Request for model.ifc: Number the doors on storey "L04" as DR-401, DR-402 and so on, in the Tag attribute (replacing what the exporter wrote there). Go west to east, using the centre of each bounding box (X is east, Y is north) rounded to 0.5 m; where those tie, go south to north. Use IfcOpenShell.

First a look at what the model holds.

```python
import ifcopenshell
import ifcopenshell.util.element
import ifcopenshell.util.placement

model = ifcopenshell.open("model.ifc")
print(model.schema)
storey = next(s for s in model.by_type("IfcBuildingStorey") if s.Name == "L04")
doors = [e for e in ifcopenshell.util.element.get_decomposition(storey) if e.is_a("IfcDoor")]
for e in sorted(doors, key=lambda e: e.id()):
    origin = ifcopenshell.util.placement.get_local_placement(e.ObjectPlacement)[:3, 3]
    print(e.id(), e.Tag, e.Name, origin.round(2) + 0.0, sep=" | ")
```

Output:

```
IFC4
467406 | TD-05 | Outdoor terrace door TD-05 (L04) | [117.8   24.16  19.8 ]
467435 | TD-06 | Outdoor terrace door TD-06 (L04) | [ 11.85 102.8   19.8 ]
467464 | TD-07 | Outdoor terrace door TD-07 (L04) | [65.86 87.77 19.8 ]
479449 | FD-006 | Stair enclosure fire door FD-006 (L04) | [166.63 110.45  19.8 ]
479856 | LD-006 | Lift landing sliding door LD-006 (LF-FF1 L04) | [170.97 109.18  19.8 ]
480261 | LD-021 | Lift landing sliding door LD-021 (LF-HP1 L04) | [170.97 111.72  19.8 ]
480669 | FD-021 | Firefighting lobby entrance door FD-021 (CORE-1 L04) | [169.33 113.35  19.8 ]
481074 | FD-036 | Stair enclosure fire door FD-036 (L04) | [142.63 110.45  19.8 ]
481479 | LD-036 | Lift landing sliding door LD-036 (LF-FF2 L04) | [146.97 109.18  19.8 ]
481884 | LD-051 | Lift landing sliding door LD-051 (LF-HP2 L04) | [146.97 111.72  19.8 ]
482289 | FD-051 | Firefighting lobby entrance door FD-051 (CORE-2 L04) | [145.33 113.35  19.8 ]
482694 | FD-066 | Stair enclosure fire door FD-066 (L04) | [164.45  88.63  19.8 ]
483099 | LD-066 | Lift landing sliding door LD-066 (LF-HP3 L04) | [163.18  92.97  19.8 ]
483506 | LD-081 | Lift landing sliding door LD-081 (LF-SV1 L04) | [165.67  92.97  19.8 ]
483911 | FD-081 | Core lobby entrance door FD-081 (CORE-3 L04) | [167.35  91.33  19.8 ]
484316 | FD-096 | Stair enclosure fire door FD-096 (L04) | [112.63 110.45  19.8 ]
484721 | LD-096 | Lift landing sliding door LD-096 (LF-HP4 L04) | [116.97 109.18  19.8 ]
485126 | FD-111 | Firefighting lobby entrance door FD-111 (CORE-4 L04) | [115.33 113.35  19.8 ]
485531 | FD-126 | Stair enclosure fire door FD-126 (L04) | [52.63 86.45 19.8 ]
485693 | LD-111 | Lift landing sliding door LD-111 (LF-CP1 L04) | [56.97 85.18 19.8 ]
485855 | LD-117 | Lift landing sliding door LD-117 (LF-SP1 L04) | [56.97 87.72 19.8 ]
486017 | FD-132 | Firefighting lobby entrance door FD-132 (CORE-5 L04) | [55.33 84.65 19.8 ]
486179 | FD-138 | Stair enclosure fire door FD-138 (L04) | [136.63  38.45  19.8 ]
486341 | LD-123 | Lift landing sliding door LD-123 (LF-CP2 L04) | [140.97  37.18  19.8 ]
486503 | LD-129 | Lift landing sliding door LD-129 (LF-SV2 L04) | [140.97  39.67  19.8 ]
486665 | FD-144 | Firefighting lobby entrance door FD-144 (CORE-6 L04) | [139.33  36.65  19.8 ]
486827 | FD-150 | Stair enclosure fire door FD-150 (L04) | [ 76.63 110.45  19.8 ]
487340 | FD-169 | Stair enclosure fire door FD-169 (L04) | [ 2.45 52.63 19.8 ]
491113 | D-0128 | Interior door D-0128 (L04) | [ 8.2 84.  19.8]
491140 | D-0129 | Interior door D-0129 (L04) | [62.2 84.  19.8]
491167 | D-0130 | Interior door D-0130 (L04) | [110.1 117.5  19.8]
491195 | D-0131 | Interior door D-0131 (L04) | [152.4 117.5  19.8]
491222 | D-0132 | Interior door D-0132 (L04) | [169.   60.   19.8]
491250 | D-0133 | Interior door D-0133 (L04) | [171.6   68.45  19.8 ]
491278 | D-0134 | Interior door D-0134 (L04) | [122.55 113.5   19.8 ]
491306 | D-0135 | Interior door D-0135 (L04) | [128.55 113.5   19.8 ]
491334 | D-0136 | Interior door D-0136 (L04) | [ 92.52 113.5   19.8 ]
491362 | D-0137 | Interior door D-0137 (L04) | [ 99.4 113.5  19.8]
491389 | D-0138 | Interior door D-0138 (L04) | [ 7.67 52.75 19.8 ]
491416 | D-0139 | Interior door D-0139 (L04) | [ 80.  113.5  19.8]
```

```python
import ifcopenshell
import ifcopenshell.geom
import ifcopenshell.util.element
import ifcopenshell.util.shape

model = ifcopenshell.open("model.ifc")
settings = ifcopenshell.geom.settings()
settings.set("use-world-coords", True)


def centre(element):
    shape = ifcopenshell.geom.create_shape(settings, element)
    return ifcopenshell.util.shape.get_bbox_centroid(shape.geometry)


storey = next(s for s in model.by_type("IfcBuildingStorey") if s.Name == "L04")
doors = [e for e in ifcopenshell.util.element.get_decomposition(storey) if e.is_a("IfcDoor")]

# Insertion points can sit at a corner or the storey origin, so sort by the geometry (in metres).
centres = {e: centre(e) for e in doors}
doors.sort(key=lambda e: (round(centres[e][0] / 0.5), centres[e][1]))

for i, e in enumerate(doors, start=1):
    number = f"DR-4{i:02d}"
    e.Tag = number
    print(e.id(), number)

model.write("model_v2.ifc")
```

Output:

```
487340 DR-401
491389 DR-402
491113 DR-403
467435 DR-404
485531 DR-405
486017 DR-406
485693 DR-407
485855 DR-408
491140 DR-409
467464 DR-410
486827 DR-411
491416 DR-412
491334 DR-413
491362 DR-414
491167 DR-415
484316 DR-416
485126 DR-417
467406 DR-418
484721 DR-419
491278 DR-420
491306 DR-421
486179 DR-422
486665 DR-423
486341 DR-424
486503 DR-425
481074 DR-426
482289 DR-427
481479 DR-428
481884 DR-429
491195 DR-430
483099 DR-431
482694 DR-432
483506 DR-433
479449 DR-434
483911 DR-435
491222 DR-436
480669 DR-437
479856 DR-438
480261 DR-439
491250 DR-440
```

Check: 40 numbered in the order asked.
